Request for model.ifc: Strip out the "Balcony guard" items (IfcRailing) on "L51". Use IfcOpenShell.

First a look at what the model holds.

```python
import ifcopenshell
import ifcopenshell.util.element

model = ifcopenshell.open("model.ifc")
print(model.schema)
storey = next(s for s in model.by_type("IfcBuildingStorey") if s.Name == "L51")
railings = [e for e in ifcopenshell.util.element.get_decomposition(storey) if e.is_a("IfcRailing")]
seen = {}
for e in railings:
    element_type = ifcopenshell.util.element.get_type(e)
    name = element_type.Name if element_type not in (None, e) else None
    seen[name] = seen.get(name, 0) + 1
for name, count in sorted(seen.items(), key=str):
    print(count, "x", name)
```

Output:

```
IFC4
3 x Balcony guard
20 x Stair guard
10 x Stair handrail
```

```python
import ifcopenshell
import ifcopenshell.api.root
import ifcopenshell.util.element

model = ifcopenshell.open("model.ifc")

storey = next(s for s in model.by_type("IfcBuildingStorey") if s.Name == "L51")
railings = [e for e in ifcopenshell.util.element.get_decomposition(storey) if e.is_a("IfcRailing")]
targets = [e for e in railings if (t := ifcopenshell.util.element.get_type(e)) not in (None, e) and t.Name == "Balcony guard"]

for e in targets:
    ifcopenshell.api.root.remove_product(model, product=e)
print(len(targets), "removed")

model.write("model_v2.ifc")
```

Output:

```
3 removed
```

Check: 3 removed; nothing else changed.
